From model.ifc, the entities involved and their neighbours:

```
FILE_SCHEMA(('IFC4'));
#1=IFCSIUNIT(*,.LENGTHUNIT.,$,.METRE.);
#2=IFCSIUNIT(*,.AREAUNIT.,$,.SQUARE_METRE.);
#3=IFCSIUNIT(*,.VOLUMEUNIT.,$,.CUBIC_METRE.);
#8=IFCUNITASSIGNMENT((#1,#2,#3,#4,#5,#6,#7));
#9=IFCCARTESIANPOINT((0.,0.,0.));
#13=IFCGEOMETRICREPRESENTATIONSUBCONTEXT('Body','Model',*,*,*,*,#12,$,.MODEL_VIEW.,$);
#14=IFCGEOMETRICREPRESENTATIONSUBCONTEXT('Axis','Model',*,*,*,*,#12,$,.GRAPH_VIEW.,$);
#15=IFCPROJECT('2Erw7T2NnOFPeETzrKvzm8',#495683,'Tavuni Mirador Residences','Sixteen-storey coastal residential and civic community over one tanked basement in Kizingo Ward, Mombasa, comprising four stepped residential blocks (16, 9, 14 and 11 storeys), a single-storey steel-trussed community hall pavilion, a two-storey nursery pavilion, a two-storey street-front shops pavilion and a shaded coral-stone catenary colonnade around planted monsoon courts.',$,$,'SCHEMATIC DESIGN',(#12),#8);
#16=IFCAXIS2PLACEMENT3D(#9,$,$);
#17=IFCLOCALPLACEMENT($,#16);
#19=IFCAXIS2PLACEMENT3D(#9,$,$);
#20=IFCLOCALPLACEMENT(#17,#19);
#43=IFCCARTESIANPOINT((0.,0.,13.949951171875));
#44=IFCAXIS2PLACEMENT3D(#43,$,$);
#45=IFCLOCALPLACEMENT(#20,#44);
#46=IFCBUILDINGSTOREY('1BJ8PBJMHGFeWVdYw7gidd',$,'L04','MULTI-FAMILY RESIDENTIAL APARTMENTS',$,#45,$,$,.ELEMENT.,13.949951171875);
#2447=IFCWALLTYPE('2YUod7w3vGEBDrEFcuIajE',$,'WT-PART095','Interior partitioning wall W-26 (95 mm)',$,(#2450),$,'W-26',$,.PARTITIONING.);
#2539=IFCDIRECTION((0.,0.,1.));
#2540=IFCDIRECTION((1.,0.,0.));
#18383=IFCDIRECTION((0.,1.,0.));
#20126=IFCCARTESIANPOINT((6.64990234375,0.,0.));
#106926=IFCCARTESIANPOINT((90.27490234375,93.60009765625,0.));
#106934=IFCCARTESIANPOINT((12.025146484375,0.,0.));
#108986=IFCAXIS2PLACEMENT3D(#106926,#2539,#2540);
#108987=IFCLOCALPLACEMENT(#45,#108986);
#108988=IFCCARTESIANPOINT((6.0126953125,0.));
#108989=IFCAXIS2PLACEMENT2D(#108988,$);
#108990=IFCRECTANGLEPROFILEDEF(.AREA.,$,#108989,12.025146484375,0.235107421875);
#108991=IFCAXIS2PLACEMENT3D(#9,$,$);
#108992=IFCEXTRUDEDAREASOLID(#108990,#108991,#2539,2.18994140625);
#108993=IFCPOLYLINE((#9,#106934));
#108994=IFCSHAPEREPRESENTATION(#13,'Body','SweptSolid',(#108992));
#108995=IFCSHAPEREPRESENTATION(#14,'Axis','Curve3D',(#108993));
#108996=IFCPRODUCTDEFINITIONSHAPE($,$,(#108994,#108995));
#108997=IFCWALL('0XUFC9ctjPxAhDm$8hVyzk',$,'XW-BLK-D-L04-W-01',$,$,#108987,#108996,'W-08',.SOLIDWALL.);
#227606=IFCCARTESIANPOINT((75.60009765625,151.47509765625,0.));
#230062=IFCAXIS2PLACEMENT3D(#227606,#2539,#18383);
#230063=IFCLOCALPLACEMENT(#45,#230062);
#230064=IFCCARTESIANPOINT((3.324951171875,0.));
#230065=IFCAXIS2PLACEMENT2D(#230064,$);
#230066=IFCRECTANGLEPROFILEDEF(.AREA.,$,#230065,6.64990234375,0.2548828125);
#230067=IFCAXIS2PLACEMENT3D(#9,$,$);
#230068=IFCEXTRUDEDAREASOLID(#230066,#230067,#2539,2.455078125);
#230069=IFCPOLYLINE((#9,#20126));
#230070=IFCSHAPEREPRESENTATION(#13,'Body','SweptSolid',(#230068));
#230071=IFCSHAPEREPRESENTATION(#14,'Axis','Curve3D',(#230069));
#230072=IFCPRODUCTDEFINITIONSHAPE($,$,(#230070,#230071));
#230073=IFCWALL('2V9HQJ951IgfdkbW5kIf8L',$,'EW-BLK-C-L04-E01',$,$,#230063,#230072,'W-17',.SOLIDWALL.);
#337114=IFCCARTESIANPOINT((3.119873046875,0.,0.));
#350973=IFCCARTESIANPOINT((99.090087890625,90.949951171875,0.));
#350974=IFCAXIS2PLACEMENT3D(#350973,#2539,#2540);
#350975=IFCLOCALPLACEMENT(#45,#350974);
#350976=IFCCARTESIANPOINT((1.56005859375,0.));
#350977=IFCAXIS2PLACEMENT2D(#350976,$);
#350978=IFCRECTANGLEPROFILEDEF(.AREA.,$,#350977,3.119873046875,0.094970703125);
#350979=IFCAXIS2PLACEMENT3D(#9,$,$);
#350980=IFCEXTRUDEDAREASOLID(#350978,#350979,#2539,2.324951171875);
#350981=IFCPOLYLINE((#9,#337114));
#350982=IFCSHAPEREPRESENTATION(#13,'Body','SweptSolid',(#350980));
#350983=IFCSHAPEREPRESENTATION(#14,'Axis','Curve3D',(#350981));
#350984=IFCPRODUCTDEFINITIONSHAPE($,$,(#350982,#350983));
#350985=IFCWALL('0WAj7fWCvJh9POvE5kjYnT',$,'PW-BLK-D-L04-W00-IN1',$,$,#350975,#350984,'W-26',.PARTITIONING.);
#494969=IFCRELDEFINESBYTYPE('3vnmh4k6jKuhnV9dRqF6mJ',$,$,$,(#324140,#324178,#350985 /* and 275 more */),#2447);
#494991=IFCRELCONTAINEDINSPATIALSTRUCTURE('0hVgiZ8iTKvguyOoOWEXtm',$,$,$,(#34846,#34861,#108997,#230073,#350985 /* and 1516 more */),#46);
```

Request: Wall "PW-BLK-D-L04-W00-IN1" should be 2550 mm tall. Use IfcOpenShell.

```python
import ifcopenshell
import ifcopenshell.geom
import ifcopenshell.util.representation
import ifcopenshell.util.shape

model = ifcopenshell.open("model.ifc")
settings = ifcopenshell.geom.settings()


def volume(element):
    """Net volume in cubic metres, openings subtracted."""
    shape = ifcopenshell.geom.create_shape(settings, element)
    return ifcopenshell.util.shape.get_volume(shape.geometry)


wall = model.by_guid("0WAj7fWCvJh9POvE5kjYnT")
before = volume(wall)

body = ifcopenshell.util.representation.get_representation(wall, "Model", "Body")
solid = body.Items[0]
old_height = solid.Depth
solid.Depth = 2.55
after = volume(wall)

print(f"height {old_height:g} -> {solid.Depth:g}, volume {before:.3f} -> {after:.3f} m3")

model.write("model_edited.ifc")
```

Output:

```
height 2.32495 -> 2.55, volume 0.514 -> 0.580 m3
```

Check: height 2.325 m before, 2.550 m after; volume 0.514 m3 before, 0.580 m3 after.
